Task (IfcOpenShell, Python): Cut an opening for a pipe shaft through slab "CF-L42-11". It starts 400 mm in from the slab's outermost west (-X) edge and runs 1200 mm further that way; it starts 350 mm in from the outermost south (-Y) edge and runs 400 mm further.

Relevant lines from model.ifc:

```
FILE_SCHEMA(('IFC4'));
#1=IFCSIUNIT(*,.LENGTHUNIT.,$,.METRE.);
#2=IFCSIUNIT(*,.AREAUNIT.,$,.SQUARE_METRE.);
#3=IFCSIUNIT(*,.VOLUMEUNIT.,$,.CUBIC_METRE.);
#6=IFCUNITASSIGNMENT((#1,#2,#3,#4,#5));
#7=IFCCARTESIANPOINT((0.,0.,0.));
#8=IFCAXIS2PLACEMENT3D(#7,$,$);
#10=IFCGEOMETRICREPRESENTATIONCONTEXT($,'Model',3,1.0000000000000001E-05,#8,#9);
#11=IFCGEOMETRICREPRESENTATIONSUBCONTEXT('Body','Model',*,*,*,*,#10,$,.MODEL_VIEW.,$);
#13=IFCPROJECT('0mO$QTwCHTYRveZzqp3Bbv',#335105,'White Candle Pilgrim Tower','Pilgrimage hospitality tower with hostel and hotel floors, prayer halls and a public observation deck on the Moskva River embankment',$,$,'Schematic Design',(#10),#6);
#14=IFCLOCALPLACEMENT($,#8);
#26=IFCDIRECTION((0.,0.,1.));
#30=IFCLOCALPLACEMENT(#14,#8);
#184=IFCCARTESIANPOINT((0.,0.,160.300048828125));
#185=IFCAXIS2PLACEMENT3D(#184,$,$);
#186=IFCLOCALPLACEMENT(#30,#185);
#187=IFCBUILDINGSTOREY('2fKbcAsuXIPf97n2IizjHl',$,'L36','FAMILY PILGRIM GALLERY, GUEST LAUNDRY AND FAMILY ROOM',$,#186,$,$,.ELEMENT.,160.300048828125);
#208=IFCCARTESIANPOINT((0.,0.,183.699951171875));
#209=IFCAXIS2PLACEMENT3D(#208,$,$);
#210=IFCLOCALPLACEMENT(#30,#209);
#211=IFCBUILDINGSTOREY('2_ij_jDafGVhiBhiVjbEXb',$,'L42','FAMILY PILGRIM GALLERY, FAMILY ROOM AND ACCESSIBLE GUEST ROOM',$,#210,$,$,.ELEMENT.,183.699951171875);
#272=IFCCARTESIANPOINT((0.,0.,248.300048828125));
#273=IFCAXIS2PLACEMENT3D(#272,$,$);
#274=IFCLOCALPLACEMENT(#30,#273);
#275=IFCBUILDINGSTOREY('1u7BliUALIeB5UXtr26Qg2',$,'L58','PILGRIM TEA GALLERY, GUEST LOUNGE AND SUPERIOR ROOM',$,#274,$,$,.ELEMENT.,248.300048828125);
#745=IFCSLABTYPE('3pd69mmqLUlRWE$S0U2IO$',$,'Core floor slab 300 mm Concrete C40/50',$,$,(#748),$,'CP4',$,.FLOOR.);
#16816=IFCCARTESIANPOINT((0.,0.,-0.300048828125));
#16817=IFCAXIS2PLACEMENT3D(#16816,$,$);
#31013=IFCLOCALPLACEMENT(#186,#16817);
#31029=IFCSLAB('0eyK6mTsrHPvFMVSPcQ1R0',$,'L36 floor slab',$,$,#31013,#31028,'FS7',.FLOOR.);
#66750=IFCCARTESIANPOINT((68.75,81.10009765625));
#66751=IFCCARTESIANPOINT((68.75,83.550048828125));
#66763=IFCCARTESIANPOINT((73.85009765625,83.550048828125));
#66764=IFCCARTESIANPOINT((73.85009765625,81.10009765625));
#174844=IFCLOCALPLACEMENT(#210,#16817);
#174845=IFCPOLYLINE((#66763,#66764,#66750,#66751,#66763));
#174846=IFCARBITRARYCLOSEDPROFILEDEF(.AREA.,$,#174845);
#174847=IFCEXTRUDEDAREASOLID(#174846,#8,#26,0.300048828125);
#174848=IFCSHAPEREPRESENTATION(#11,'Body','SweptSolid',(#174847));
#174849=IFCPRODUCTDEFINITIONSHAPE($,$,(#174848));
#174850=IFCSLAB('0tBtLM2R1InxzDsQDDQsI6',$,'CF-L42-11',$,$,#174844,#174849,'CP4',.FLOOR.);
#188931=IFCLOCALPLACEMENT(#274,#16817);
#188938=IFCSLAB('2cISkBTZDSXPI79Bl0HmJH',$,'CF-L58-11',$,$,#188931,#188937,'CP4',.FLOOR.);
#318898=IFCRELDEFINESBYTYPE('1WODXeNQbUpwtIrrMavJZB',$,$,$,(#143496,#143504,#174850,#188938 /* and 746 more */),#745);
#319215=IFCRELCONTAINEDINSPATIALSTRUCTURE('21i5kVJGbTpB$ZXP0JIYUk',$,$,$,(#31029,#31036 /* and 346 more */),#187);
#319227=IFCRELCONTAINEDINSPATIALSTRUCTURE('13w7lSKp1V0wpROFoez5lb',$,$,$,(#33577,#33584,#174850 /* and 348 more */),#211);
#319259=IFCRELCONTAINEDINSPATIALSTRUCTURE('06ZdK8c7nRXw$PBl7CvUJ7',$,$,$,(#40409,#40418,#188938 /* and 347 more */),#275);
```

```python
import numpy as np
import ifcopenshell
import ifcopenshell.api.feature
import ifcopenshell.api.geometry
import ifcopenshell.api.root
import ifcopenshell.geom
import ifcopenshell.util.placement
import ifcopenshell.util.representation
import ifcopenshell.util.shape
import ifcopenshell.util.unit

model = ifcopenshell.open("model.ifc")
unit_scale = ifcopenshell.util.unit.calculate_unit_scale(model)
settings = ifcopenshell.geom.settings()


def volume(element):
    """Net volume in cubic metres, openings subtracted."""
    shape = ifcopenshell.geom.create_shape(settings, element)
    return ifcopenshell.util.shape.get_volume(shape.geometry)


slab = model.by_guid("0tBtLM2R1InxzDsQDDQsI6")
before = volume(slab)

# Extent in the slab's own axes, in metres. The edges named are its -X and -Y sides.
slab_shape = ifcopenshell.geom.create_shape(settings, slab)
vertices = ifcopenshell.util.shape.get_vertices(slab_shape.geometry)
x_min, y_min, bottom = vertices.min(axis=0)
top = vertices[:, 2].max()

opening = ifcopenshell.api.root.create_entity(model, ifc_class="IfcOpeningElement", name="Pipe shaft opening", predefined_type="OPENING")
context = ifcopenshell.util.representation.get_context(model, "Model", "Body", "MODEL_VIEW")
width, depth = 1.2, 0.4
outline = [(0.0, 0.0), (width, 0.0), (width, depth), (0.0, depth), (0.0, 0.0)]
# Overshoot both faces by 50 mm so the cut is clean.
shape = ifcopenshell.api.geometry.add_slab_representation(
    model, context=context, depth=top - bottom + 0.1, polyline=outline
)
ifcopenshell.api.geometry.assign_representation(model, product=opening, representation=shape)

matrix = ifcopenshell.util.placement.get_local_placement(slab.ObjectPlacement)
matrix[:, 3] = matrix @ np.append(np.array([x_min + 0.4, y_min + 0.35, bottom - 0.05]) / unit_scale, 1.0)
ifcopenshell.api.geometry.edit_object_placement(model, product=opening, matrix=matrix, is_si=False)
ifcopenshell.api.feature.add_feature(model, feature=opening, element=slab)

after = volume(slab)

print(f"slab volume {before:.3f} -> {after:.3f} m3")

model.write("model_rev.ifc")
```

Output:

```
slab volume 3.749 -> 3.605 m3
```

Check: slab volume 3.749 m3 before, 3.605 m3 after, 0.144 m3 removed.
